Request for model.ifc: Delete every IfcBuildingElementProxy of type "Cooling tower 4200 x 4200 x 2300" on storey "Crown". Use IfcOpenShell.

First a look at what the model holds.

```python
import ifcopenshell
import ifcopenshell.util.element

model = ifcopenshell.open("model.ifc")
print(model.schema)
storey = next(s for s in model.by_type("IfcBuildingStorey") if s.Name == "Crown")
proxies = [e for e in ifcopenshell.util.element.get_decomposition(storey) if e.is_a("IfcBuildingElementProxy")]
seen = {}
for e in proxies:
    element_type = ifcopenshell.util.element.get_type(e)
    name = element_type.Name if element_type not in (None, e) else None
    seen[name] = seen.get(name, 0) + 1
for name, count in sorted(seen.items(), key=str):
    print(count, "x", name)
```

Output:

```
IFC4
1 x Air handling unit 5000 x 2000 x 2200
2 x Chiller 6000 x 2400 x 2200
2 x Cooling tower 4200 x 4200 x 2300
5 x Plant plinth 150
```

```python
import ifcopenshell
import ifcopenshell.api.root
import ifcopenshell.util.element

model = ifcopenshell.open("model.ifc")

storey = next(s for s in model.by_type("IfcBuildingStorey") if s.Name == "Crown")
proxies = [e for e in ifcopenshell.util.element.get_decomposition(storey) if e.is_a("IfcBuildingElementProxy")]
targets = [e for e in proxies if (t := ifcopenshell.util.element.get_type(e)) not in (None, e) and t.Name == "Cooling tower 4200 x 4200 x 2300"]

for e in targets:
    ifcopenshell.api.root.remove_product(model, product=e)
print(len(targets), "removed")

model.write("model_edited.ifc")
```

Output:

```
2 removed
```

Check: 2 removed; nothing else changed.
